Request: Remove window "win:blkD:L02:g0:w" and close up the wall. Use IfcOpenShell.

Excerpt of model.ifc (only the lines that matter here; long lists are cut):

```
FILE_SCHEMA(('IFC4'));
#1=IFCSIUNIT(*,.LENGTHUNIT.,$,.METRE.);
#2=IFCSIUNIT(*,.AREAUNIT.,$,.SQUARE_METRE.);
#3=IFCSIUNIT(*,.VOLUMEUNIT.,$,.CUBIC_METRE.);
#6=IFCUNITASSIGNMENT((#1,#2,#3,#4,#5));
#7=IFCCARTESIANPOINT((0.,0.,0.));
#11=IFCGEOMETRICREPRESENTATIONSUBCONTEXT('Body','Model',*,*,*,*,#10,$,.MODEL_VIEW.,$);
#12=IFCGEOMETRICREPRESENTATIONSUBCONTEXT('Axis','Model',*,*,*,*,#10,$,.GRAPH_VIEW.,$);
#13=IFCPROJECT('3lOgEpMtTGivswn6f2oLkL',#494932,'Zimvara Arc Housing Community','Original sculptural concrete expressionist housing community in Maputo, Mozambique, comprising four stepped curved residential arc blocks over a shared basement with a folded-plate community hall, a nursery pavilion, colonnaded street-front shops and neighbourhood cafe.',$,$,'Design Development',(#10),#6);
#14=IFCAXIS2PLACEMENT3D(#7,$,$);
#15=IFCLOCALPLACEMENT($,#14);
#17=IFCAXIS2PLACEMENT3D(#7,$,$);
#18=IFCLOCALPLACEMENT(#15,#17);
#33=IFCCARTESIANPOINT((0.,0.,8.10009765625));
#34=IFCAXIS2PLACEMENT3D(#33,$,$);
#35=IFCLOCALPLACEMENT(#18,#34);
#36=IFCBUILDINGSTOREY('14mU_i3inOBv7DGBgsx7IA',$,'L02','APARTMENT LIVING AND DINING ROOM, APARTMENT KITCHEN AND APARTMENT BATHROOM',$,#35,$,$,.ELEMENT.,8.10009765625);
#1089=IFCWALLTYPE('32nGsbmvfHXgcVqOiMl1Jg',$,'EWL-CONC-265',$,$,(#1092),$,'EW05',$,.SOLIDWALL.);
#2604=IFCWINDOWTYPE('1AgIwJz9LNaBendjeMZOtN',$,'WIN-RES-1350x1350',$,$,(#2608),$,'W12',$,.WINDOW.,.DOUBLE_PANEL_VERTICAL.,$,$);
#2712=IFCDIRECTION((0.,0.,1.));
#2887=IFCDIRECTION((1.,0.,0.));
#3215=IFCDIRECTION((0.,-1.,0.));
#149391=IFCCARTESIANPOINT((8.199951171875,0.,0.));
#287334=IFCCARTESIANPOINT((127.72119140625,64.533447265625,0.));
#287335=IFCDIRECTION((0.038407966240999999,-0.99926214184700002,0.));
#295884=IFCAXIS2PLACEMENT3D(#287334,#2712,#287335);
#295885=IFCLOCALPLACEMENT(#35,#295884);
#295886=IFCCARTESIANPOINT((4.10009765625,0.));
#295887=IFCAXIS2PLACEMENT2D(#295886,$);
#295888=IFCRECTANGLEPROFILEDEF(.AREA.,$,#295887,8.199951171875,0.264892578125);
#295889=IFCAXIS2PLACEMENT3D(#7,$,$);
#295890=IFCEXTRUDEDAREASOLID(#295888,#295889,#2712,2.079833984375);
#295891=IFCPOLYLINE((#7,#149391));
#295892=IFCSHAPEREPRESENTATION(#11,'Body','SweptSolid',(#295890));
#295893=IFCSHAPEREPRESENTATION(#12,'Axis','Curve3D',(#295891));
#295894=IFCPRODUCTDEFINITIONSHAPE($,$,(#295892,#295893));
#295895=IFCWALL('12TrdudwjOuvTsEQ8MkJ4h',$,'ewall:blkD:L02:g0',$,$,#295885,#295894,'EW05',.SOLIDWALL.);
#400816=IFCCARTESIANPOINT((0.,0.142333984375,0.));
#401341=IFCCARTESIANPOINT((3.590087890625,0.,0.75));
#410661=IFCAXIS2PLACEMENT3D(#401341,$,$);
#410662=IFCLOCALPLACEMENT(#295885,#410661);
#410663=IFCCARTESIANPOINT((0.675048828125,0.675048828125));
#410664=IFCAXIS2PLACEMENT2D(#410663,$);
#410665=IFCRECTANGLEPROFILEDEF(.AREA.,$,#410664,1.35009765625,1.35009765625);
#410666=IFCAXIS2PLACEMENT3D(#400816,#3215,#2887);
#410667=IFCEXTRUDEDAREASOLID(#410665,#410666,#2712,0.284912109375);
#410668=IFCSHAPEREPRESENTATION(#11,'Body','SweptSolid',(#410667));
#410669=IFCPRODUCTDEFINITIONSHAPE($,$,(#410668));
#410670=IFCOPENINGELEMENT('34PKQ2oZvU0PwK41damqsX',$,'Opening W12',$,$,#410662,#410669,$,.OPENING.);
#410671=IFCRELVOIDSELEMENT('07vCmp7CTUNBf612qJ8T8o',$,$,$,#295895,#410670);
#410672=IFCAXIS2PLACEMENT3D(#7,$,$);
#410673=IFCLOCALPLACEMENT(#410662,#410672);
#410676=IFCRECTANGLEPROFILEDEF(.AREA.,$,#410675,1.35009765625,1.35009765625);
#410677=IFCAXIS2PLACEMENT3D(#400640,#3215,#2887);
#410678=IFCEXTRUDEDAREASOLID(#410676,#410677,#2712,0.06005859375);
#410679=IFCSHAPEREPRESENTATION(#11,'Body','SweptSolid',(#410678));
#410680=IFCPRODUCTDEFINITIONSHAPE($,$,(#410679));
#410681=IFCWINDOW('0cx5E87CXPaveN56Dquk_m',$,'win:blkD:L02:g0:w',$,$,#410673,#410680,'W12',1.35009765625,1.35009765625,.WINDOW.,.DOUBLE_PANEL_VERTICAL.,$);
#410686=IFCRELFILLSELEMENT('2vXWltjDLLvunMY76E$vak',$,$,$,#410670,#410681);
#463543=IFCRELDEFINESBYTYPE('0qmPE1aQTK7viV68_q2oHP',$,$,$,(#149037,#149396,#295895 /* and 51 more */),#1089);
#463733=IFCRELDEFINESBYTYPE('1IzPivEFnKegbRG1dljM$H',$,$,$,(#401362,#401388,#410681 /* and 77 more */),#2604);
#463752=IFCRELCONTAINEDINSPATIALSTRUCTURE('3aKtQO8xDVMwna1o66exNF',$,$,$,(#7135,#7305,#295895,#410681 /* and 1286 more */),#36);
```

```python
import ifcopenshell
import ifcopenshell.api.feature
import ifcopenshell.api.root
import ifcopenshell.geom
import ifcopenshell.util.shape

model = ifcopenshell.open("model.ifc")
settings = ifcopenshell.geom.settings()


def volume(element):
    """Net volume in cubic metres, openings subtracted."""
    shape = ifcopenshell.geom.create_shape(settings, element)
    return ifcopenshell.util.shape.get_volume(shape.geometry)


window = model.by_guid("0cx5E87CXPaveN56Dquk_m")
opening = window.FillsVoids[0].RelatingOpeningElement
wall = opening.VoidsElements[0].RelatingBuildingElement
before = volume(wall)

ifcopenshell.api.root.remove_product(model, product=window)
ifcopenshell.api.feature.remove_feature(model, feature=opening)

after = volume(wall)

print(f"wall volume {before:.3f} -> {after:.3f} m3")

model.write("model-out.ifc")
```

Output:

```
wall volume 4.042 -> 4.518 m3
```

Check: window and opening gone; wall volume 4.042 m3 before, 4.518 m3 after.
